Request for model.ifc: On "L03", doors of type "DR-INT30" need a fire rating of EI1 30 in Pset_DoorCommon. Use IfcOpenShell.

First a look at what the model holds.

```python
import ifcopenshell
import ifcopenshell.util.element

model = ifcopenshell.open("model.ifc")
print(model.schema)
storey = next(s for s in model.by_type("IfcBuildingStorey") if s.Name == "L03")
doors = [e for e in ifcopenshell.util.element.get_decomposition(storey) if e.is_a("IfcDoor")]
seen = {}
for e in doors:
    element_type = ifcopenshell.util.element.get_type(e)
    key = (element_type.Name if element_type != e and element_type else None, ifcopenshell.util.element.get_pset(e, "Pset_DoorCommon", "FireRating"))
    seen[key] = seen.get(key, 0) + 1
for (name, value), count in sorted(seen.items(), key=str):
    print(count, "x", name, "|", value)
```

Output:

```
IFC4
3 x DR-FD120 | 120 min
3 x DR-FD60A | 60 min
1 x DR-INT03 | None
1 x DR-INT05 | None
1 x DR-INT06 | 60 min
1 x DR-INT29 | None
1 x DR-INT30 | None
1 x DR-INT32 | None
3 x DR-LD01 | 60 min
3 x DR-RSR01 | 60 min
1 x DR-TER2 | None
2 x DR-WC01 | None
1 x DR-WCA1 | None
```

```python
import ifcopenshell
import ifcopenshell.api.pset
import ifcopenshell.util.element

model = ifcopenshell.open("model.ifc")

storey = next(s for s in model.by_type("IfcBuildingStorey") if s.Name == "L03")
doors = [e for e in ifcopenshell.util.element.get_decomposition(storey) if e.is_a("IfcDoor")]

count = 0
for e in doors:
    element_type = ifcopenshell.util.element.get_type(e)
    if element_type in (None, e) or element_type.Name != "DR-INT30":
        continue
    # add_pset returns the element's existing set when there is one.
    pset = ifcopenshell.api.pset.add_pset(model, product=e, name="Pset_DoorCommon")
    ifcopenshell.api.pset.edit_pset(model, pset=pset, properties={"FireRating": "EI1 30"})
    count += 1

print(count, "doors updated")

model.write("model_edited.ifc")
```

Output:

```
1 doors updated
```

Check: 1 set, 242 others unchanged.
